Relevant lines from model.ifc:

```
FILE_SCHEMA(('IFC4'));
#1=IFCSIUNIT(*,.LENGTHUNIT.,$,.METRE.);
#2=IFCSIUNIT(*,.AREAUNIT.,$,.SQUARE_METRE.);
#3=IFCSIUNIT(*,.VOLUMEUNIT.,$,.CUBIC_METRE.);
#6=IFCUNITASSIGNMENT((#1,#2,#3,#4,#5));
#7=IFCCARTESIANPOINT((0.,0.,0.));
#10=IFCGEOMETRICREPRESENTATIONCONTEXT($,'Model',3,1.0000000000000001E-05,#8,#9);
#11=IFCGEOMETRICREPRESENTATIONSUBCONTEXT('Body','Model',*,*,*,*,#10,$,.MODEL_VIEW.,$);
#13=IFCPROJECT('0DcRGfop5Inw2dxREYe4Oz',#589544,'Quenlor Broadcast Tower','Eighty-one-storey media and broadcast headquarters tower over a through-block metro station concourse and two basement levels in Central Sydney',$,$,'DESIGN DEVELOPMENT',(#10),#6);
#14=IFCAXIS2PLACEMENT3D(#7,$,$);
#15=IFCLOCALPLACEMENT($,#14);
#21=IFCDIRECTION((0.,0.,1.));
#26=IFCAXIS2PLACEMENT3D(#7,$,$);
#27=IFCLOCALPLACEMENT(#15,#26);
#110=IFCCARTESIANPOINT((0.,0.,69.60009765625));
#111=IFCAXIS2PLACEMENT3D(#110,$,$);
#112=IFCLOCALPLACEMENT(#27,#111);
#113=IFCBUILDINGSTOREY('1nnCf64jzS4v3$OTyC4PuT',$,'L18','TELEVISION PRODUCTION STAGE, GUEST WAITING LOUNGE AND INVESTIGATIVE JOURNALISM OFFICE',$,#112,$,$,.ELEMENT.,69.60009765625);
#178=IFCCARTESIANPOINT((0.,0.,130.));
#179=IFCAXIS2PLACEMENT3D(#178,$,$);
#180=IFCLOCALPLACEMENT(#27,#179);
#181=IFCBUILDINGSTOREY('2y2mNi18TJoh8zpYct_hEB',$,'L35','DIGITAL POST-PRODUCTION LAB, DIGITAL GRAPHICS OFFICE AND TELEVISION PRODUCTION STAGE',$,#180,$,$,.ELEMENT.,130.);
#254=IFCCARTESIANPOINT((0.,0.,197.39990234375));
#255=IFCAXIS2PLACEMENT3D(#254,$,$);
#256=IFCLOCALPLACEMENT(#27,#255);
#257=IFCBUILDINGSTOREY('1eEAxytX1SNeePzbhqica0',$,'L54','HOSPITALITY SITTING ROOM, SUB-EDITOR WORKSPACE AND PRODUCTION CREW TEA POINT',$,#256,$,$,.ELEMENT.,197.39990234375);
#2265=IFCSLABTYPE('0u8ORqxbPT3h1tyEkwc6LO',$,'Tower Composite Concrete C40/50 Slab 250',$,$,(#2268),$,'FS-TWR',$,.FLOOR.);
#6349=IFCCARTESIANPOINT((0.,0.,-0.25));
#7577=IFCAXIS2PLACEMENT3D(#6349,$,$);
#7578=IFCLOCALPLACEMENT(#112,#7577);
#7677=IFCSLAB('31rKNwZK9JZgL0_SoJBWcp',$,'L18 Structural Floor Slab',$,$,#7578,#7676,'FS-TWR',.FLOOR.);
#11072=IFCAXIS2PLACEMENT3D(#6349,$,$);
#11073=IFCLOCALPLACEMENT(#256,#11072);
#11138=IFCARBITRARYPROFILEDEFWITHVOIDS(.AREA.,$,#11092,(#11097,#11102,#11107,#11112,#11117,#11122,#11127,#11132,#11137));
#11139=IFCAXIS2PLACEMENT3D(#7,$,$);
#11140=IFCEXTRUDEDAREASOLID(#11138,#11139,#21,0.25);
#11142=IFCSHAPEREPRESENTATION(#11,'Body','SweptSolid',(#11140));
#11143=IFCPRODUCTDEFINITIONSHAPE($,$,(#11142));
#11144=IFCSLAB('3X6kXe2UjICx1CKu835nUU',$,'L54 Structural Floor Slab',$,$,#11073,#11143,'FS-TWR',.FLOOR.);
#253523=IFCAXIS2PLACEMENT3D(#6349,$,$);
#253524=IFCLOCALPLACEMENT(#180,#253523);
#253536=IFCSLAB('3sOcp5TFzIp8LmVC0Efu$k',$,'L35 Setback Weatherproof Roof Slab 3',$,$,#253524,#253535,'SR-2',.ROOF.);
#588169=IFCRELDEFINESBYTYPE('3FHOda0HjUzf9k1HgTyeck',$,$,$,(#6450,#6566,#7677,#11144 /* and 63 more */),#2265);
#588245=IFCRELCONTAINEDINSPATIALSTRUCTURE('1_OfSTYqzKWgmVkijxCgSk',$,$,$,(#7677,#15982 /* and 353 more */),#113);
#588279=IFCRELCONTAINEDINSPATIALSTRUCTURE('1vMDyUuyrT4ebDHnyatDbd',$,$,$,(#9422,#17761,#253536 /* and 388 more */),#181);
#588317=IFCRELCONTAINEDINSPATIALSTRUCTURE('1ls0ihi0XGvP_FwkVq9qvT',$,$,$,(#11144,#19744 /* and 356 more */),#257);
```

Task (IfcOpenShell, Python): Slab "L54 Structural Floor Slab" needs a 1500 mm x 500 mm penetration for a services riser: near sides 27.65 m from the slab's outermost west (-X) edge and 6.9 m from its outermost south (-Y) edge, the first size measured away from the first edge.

```python
import numpy as np
import ifcopenshell
import ifcopenshell.api.feature
import ifcopenshell.api.geometry
import ifcopenshell.api.root
import ifcopenshell.geom
import ifcopenshell.util.placement
import ifcopenshell.util.representation
import ifcopenshell.util.shape
import ifcopenshell.util.unit

model = ifcopenshell.open("model.ifc")
unit_scale = ifcopenshell.util.unit.calculate_unit_scale(model)
settings = ifcopenshell.geom.settings()


def volume(element):
    """Net volume in cubic metres, openings subtracted."""
    shape = ifcopenshell.geom.create_shape(settings, element)
    return ifcopenshell.util.shape.get_volume(shape.geometry)


slab = model.by_guid("3X6kXe2UjICx1CKu835nUU")
before = volume(slab)

# Extent in the slab's own axes, in metres. The edges named are its -X and -Y sides.
slab_shape = ifcopenshell.geom.create_shape(settings, slab)
vertices = ifcopenshell.util.shape.get_vertices(slab_shape.geometry)
x_min, y_min, bottom = vertices.min(axis=0)
top = vertices[:, 2].max()

opening = ifcopenshell.api.root.create_entity(model, ifc_class="IfcOpeningElement", name="Services riser opening", predefined_type="OPENING")
context = ifcopenshell.util.representation.get_context(model, "Model", "Body", "MODEL_VIEW")
width, depth = 1.5, 0.5
outline = [(0.0, 0.0), (width, 0.0), (width, depth), (0.0, depth), (0.0, 0.0)]
# Overshoot both faces by 50 mm so the cut is clean.
shape = ifcopenshell.api.geometry.add_slab_representation(
    model, context=context, depth=top - bottom + 0.1, polyline=outline
)
ifcopenshell.api.geometry.assign_representation(model, product=opening, representation=shape)

matrix = ifcopenshell.util.placement.get_local_placement(slab.ObjectPlacement)
matrix[:, 3] = matrix @ np.append(np.array([x_min + 27.65, y_min + 6.9, bottom - 0.05]) / unit_scale, 1.0)
ifcopenshell.api.geometry.edit_object_placement(model, product=opening, matrix=matrix, is_si=False)
ifcopenshell.api.feature.add_feature(model, feature=opening, element=slab)

after = volume(slab)

print(f"slab volume {before:.3f} -> {after:.3f} m3")

model.write("model-out.ifc")
```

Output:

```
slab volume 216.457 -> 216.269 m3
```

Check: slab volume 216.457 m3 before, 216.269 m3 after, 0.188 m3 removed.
